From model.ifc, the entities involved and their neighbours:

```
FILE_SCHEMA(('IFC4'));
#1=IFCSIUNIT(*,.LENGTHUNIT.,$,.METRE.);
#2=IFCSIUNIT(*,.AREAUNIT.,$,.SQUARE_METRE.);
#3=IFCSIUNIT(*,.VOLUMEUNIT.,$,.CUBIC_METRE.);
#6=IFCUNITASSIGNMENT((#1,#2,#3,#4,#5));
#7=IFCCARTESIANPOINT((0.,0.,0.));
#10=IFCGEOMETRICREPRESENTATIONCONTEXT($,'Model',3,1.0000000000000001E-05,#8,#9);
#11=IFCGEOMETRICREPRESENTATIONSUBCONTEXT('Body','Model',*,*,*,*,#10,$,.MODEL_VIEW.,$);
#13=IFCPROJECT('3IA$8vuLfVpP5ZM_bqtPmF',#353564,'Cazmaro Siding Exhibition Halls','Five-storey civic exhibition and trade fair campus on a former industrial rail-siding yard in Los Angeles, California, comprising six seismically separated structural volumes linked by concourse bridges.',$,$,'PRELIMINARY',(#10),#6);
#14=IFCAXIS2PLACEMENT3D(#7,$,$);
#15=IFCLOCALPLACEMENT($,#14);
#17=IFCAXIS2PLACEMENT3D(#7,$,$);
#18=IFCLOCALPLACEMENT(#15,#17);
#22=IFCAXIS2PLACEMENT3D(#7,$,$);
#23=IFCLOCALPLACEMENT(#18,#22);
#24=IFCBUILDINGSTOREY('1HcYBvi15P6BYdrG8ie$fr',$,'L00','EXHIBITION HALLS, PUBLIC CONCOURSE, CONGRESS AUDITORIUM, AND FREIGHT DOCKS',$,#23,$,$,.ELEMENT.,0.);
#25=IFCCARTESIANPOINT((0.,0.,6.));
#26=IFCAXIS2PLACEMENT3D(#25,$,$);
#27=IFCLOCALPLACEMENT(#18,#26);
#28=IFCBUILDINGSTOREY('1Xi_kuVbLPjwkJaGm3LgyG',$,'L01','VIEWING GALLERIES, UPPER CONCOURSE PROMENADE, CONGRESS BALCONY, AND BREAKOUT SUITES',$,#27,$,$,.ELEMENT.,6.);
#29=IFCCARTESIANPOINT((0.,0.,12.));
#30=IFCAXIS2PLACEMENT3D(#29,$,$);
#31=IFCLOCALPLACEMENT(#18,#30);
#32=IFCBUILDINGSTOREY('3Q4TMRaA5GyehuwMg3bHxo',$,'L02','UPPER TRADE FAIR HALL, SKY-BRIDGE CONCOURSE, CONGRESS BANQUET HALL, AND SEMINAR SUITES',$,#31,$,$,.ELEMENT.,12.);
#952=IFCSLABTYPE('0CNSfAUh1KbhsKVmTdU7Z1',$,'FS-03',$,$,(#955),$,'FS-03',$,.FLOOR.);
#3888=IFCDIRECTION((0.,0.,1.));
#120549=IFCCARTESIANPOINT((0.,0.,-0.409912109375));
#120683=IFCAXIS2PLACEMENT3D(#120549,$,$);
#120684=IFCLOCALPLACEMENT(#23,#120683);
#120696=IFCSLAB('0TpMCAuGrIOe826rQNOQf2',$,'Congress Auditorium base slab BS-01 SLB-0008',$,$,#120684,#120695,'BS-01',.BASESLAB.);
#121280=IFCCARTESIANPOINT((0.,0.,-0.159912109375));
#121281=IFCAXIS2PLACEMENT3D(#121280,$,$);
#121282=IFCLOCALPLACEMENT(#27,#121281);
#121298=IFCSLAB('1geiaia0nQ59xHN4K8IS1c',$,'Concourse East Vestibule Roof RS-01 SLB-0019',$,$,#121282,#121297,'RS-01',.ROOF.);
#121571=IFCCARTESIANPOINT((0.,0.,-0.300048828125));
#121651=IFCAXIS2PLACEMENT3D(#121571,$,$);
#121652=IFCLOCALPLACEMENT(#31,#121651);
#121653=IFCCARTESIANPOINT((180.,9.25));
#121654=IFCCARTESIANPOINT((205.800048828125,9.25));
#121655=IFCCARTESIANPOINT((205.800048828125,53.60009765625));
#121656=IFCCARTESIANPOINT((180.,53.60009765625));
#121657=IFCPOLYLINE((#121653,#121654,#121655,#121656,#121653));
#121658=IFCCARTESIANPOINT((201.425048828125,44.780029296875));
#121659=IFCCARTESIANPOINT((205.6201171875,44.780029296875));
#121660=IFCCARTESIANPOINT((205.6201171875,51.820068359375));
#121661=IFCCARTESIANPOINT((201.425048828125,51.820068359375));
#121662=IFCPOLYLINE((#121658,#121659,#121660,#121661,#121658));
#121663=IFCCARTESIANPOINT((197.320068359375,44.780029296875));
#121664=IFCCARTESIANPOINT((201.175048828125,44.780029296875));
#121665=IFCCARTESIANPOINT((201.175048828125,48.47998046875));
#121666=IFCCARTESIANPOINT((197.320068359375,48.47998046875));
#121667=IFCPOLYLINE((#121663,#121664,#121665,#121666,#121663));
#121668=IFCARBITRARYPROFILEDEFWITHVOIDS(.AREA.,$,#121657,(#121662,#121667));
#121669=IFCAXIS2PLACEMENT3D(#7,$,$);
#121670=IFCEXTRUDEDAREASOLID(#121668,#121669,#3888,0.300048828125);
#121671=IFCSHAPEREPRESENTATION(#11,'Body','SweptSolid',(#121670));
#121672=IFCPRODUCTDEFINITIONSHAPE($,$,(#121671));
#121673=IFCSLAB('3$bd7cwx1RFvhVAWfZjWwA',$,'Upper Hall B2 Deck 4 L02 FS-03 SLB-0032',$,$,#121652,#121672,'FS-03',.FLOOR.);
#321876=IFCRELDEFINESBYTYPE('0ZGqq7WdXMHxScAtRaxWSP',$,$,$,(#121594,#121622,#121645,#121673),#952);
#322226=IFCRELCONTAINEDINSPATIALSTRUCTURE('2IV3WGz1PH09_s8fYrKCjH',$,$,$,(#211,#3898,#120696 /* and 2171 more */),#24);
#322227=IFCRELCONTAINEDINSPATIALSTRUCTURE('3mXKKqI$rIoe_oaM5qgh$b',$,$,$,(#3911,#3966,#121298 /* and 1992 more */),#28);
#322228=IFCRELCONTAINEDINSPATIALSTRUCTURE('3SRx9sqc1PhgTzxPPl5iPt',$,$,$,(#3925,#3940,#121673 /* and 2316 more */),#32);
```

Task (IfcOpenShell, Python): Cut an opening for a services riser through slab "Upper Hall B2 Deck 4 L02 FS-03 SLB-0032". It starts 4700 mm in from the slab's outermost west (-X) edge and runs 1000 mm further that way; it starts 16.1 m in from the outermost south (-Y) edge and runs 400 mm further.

```python
import numpy as np
import ifcopenshell
import ifcopenshell.api.feature
import ifcopenshell.api.geometry
import ifcopenshell.api.root
import ifcopenshell.geom
import ifcopenshell.util.placement
import ifcopenshell.util.representation
import ifcopenshell.util.shape
import ifcopenshell.util.unit

model = ifcopenshell.open("model.ifc")
unit_scale = ifcopenshell.util.unit.calculate_unit_scale(model)
settings = ifcopenshell.geom.settings()


def volume(element):
    """Net volume in cubic metres, openings subtracted."""
    shape = ifcopenshell.geom.create_shape(settings, element)
    return ifcopenshell.util.shape.get_volume(shape.geometry)


slab = model.by_guid("3$bd7cwx1RFvhVAWfZjWwA")
before = volume(slab)

# Extent in the slab's own axes, in metres. The edges named are its -X and -Y sides.
slab_shape = ifcopenshell.geom.create_shape(settings, slab)
vertices = ifcopenshell.util.shape.get_vertices(slab_shape.geometry)
x_min, y_min, bottom = vertices.min(axis=0)
top = vertices[:, 2].max()

opening = ifcopenshell.api.root.create_entity(model, ifc_class="IfcOpeningElement", name="Services riser opening", predefined_type="OPENING")
context = ifcopenshell.util.representation.get_context(model, "Model", "Body", "MODEL_VIEW")
width, depth = 1, 0.4
outline = [(0.0, 0.0), (width, 0.0), (width, depth), (0.0, depth), (0.0, 0.0)]
# Overshoot both faces by 50 mm so the cut is clean.
shape = ifcopenshell.api.geometry.add_slab_representation(
    model, context=context, depth=top - bottom + 0.1, polyline=outline
)
ifcopenshell.api.geometry.assign_representation(model, product=opening, representation=shape)

matrix = ifcopenshell.util.placement.get_local_placement(slab.ObjectPlacement)
matrix[:, 3] = matrix @ np.append(np.array([x_min + 4.7, y_min + 16.1, bottom - 0.05]) / unit_scale, 1.0)
ifcopenshell.api.geometry.edit_object_placement(model, product=opening, matrix=matrix, is_si=False)
ifcopenshell.api.feature.add_feature(model, feature=opening, element=slab)

after = volume(slab)

print(f"slab volume {before:.3f} -> {after:.3f} m3")

model.write("model_edited.ifc")
```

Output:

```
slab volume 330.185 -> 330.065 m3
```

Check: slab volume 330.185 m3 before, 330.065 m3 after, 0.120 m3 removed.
